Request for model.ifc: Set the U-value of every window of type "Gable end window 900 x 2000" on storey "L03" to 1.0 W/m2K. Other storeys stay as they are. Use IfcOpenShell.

First a look at what the model holds.

```python
import ifcopenshell
import ifcopenshell.util.element

model = ifcopenshell.open("model.ifc")
print(model.schema)
storey = next(s for s in model.by_type("IfcBuildingStorey") if s.Name == "L03")
windows = [e for e in ifcopenshell.util.element.get_decomposition(storey) if e.is_a("IfcWindow")]
seen = {}
for e in windows:
    element_type = ifcopenshell.util.element.get_type(e)
    key = (element_type.Name if element_type != e and element_type else None, ifcopenshell.util.element.get_pset(e, "Pset_WindowCommon", "ThermalTransmittance"))
    seen[key] = seen.get(key, 0) + 1
for (name, value), count in sorted(seen.items(), key=str):
    print(count, "x", name, "|", value)
```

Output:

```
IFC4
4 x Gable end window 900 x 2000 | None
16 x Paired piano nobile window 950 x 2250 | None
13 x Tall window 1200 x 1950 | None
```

```python
import ifcopenshell
import ifcopenshell.api.pset
import ifcopenshell.util.element

model = ifcopenshell.open("model.ifc")

storey = next(s for s in model.by_type("IfcBuildingStorey") if s.Name == "L03")
windows = [e for e in ifcopenshell.util.element.get_decomposition(storey) if e.is_a("IfcWindow")]

count = 0
for e in windows:
    element_type = ifcopenshell.util.element.get_type(e)
    if element_type in (None, e) or element_type.Name != "Gable end window 900 x 2000":
        continue
    # add_pset returns the element's existing set when there is one.
    pset = ifcopenshell.api.pset.add_pset(model, product=e, name="Pset_WindowCommon")
    ifcopenshell.api.pset.edit_pset(model, pset=pset, properties={"ThermalTransmittance": 1.0})
    count += 1

print(count, "windows updated")

model.write("model_v2.ifc")
```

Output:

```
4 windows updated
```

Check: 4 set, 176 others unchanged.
